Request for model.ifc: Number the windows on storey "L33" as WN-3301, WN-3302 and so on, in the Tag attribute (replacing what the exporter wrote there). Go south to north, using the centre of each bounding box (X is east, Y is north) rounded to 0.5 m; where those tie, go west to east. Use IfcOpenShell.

First a look at what the model holds.

```python
import ifcopenshell
import ifcopenshell.util.element
import ifcopenshell.util.placement

model = ifcopenshell.open("model.ifc")
print(model.schema)
storey = next(s for s in model.by_type("IfcBuildingStorey") if s.Name == "L33")
windows = [e for e in ifcopenshell.util.element.get_decomposition(storey) if e.is_a("IfcWindow")]
for e in sorted(windows, key=lambda e: e.id()):
    origin = ifcopenshell.util.placement.get_local_placement(e.ObjectPlacement)[:3, 3]
    print(e.id(), e.Tag, e.Name, origin.round(2) + 0.0, sep=" | ")
```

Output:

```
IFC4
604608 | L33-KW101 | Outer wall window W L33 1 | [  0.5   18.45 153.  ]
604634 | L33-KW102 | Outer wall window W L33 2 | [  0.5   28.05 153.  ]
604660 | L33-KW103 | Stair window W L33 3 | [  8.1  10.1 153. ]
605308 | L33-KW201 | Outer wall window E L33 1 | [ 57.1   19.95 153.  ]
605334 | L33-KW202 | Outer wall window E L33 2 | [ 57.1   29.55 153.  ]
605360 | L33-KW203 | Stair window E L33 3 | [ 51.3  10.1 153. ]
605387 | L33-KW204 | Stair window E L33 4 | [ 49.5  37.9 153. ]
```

```python
import ifcopenshell
import ifcopenshell.geom
import ifcopenshell.util.element
import ifcopenshell.util.shape

model = ifcopenshell.open("model.ifc")
settings = ifcopenshell.geom.settings()
settings.set("use-world-coords", True)


def centre(element):
    shape = ifcopenshell.geom.create_shape(settings, element)
    return ifcopenshell.util.shape.get_bbox_centroid(shape.geometry)


storey = next(s for s in model.by_type("IfcBuildingStorey") if s.Name == "L33")
windows = [e for e in ifcopenshell.util.element.get_decomposition(storey) if e.is_a("IfcWindow")]

# Insertion points can sit at a corner or the storey origin, so sort by the geometry (in metres).
centres = {e: centre(e) for e in windows}
windows.sort(key=lambda e: (round(centres[e][1] / 0.5), centres[e][0]))

for i, e in enumerate(windows, start=1):
    number = f"WN-33{i:02d}"
    e.Tag = number
    print(e.id(), number)

model.write("model_edited.ifc")
```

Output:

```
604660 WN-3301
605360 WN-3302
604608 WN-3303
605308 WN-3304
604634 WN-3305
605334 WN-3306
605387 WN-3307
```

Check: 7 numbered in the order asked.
